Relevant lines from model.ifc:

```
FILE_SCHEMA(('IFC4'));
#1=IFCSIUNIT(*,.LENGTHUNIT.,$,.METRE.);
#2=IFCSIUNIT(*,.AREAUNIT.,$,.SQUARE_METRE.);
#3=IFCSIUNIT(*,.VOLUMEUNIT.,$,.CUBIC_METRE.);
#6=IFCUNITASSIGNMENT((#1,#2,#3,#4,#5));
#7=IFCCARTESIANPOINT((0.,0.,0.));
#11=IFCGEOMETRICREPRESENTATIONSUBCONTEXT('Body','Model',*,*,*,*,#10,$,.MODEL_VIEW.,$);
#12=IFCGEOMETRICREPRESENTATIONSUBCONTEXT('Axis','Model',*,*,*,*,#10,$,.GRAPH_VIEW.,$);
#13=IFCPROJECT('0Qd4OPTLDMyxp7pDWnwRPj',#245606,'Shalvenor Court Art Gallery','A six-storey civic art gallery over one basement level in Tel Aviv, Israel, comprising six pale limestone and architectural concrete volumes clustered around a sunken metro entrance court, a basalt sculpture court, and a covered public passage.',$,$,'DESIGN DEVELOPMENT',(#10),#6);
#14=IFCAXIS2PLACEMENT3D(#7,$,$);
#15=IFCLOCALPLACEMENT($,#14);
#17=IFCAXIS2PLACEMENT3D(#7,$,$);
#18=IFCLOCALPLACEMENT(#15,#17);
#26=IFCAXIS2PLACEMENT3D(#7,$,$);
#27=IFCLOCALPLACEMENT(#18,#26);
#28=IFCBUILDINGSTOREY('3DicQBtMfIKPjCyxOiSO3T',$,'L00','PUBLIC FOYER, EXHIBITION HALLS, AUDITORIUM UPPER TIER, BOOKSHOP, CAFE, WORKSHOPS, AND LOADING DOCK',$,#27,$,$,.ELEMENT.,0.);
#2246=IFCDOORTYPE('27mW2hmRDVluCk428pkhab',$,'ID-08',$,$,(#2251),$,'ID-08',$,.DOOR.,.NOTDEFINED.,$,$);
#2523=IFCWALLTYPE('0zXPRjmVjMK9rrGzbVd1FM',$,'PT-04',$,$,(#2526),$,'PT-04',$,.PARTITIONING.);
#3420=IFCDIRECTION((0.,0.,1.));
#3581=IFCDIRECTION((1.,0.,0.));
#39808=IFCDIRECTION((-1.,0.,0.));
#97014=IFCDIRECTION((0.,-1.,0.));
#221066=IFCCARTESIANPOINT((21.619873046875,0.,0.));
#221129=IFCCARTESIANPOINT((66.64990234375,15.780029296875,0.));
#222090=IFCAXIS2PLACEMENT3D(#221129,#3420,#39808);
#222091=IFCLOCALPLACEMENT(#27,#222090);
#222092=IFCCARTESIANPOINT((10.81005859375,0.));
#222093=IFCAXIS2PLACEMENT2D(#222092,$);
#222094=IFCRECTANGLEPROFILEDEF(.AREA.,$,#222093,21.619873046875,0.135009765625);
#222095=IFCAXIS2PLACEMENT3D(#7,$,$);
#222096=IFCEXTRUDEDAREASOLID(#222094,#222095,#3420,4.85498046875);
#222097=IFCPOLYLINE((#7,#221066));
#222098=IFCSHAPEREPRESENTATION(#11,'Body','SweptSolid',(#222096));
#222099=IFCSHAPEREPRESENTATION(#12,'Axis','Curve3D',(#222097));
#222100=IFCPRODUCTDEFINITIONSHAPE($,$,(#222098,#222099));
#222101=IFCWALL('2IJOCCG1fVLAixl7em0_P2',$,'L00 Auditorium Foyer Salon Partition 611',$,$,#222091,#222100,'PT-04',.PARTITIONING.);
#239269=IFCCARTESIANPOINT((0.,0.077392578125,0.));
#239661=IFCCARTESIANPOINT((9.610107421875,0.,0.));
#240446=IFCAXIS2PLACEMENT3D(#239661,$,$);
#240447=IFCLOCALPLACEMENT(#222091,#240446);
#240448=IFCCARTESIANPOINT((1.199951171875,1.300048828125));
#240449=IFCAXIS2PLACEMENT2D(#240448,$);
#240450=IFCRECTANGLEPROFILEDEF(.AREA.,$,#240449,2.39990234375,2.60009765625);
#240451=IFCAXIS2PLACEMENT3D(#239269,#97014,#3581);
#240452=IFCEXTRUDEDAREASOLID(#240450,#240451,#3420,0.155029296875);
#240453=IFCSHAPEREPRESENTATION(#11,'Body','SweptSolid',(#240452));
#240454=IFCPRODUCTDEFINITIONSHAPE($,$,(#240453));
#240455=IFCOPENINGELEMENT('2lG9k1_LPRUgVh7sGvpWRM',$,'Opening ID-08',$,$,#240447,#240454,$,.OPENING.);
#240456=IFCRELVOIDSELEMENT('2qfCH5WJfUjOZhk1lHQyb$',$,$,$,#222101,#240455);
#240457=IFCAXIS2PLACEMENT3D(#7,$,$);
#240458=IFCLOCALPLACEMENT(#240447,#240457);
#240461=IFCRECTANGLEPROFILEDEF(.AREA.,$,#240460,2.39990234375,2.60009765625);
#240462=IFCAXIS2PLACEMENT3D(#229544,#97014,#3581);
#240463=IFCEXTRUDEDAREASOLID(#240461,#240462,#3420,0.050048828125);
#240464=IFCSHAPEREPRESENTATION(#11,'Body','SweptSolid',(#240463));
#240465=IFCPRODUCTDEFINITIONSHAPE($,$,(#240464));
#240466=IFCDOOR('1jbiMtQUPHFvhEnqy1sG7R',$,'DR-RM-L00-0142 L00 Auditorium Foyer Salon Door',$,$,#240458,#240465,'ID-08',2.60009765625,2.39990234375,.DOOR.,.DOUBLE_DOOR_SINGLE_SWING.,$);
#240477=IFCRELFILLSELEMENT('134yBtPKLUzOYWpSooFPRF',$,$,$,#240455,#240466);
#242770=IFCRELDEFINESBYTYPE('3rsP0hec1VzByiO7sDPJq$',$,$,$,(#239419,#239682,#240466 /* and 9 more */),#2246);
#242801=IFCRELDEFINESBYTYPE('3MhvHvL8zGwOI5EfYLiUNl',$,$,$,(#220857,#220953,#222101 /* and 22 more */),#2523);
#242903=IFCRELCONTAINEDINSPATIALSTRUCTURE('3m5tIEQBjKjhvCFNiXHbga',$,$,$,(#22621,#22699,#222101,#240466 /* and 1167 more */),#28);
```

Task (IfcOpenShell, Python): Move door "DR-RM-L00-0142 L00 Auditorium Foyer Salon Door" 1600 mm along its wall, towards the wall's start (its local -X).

```python
import ifcopenshell
import ifcopenshell.api.geometry
import ifcopenshell.util.placement
import ifcopenshell.util.unit

model = ifcopenshell.open("model.ifc")
unit_scale = ifcopenshell.util.unit.calculate_unit_scale(model)

door = model.by_id(240466)
opening = door.FillsVoids[0].RelatingOpeningElement
wall = opening.VoidsElements[0].RelatingBuildingElement

wall_matrix = ifcopenshell.util.placement.get_local_placement(wall.ObjectPlacement)
shift = wall_matrix[:3, 0] * -1.6 / unit_scale
before = ifcopenshell.util.placement.get_local_placement(door.ObjectPlacement)[:3, 3].copy()

# The door is placed relative to its opening, so it follows when the opening moves.
matrix = ifcopenshell.util.placement.get_local_placement(opening.ObjectPlacement)
matrix[:3, 3] += shift
ifcopenshell.api.geometry.edit_object_placement(
    model, product=opening, matrix=matrix, is_si=False, should_transform_children=True
)

after = ifcopenshell.util.placement.get_local_placement(door.ObjectPlacement)[:3, 3]
print("door moved by", (after - before).round(3) + 0.0)

model.write("model_updated.ifc")
```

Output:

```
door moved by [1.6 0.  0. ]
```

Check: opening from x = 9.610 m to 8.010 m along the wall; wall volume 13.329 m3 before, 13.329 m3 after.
